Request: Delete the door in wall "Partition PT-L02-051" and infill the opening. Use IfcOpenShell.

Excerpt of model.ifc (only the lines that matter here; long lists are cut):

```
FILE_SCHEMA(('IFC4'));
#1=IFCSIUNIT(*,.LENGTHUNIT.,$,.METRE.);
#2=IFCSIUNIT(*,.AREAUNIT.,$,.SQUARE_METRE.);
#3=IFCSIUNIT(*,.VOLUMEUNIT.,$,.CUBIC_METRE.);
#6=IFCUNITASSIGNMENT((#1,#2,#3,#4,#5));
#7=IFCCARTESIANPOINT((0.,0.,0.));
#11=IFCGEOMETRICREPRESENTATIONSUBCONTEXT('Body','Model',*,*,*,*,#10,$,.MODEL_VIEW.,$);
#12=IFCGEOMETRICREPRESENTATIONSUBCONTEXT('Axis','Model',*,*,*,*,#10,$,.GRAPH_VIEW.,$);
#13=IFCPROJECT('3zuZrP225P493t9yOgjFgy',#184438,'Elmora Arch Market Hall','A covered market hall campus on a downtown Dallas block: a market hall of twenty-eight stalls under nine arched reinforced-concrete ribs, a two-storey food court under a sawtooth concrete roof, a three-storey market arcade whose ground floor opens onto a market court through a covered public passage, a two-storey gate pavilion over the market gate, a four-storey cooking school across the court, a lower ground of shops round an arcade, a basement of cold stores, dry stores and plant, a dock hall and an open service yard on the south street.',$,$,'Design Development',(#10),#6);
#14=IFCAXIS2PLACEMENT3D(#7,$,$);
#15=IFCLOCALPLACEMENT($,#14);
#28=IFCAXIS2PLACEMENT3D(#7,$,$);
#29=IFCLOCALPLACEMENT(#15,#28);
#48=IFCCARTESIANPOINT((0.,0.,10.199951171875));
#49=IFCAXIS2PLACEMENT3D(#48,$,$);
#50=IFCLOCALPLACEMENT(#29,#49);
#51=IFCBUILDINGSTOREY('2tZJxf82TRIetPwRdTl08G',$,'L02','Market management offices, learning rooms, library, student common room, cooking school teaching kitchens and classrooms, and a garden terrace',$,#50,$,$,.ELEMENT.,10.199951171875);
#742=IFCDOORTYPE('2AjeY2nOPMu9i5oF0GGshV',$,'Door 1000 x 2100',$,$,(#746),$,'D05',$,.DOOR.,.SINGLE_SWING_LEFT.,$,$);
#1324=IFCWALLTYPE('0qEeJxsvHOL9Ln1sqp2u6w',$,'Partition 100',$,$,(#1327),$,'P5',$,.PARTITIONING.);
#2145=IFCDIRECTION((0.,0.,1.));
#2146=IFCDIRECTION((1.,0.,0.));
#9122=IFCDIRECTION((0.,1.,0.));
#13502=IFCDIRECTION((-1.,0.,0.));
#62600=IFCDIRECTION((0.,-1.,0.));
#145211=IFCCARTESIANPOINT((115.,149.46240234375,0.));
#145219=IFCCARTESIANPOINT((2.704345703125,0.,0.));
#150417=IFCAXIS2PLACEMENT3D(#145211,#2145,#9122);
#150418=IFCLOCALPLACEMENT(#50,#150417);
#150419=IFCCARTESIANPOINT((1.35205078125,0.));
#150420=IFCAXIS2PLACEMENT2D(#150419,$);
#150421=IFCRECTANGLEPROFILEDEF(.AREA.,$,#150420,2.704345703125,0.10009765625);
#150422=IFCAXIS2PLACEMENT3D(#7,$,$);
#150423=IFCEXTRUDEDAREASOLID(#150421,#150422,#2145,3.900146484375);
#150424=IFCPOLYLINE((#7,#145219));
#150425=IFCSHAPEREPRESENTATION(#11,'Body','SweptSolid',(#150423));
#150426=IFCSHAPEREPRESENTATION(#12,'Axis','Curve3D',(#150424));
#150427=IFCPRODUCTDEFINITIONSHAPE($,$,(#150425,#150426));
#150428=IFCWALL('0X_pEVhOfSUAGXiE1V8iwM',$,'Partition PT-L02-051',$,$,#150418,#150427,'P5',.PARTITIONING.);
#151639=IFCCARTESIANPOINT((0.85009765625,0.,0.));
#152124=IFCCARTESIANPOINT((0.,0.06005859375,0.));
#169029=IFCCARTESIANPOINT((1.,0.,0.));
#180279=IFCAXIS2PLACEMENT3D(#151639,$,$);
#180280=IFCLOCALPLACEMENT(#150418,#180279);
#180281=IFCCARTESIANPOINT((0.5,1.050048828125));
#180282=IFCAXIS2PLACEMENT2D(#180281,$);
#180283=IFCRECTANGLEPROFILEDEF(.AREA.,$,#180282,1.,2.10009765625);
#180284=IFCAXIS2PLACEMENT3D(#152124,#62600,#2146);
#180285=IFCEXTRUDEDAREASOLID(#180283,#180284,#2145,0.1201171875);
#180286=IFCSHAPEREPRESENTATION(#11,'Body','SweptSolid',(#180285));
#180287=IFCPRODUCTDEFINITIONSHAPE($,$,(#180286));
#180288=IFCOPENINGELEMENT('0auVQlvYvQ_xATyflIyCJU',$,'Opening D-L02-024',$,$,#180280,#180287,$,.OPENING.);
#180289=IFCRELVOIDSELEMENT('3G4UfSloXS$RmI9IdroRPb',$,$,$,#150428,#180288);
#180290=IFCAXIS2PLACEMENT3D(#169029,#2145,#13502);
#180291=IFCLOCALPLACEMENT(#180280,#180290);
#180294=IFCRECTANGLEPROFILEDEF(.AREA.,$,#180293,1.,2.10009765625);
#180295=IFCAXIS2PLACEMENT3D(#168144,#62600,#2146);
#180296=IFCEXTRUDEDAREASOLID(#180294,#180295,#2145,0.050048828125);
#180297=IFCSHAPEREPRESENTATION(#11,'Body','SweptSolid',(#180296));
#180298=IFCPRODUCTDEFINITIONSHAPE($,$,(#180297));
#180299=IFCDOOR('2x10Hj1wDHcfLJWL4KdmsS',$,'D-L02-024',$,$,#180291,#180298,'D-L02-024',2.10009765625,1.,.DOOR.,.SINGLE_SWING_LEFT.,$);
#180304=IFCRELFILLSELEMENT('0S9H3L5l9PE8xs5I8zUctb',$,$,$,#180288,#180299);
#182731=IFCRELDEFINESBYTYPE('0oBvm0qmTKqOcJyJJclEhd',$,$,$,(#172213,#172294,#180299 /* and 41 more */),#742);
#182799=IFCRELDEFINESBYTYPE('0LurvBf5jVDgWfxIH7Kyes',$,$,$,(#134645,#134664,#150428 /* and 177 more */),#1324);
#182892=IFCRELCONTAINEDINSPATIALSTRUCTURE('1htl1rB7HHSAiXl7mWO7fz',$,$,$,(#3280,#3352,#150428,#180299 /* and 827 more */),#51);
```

```python
import ifcopenshell
import ifcopenshell.api.feature
import ifcopenshell.api.root
import ifcopenshell.geom
import ifcopenshell.util.shape

model = ifcopenshell.open("model.ifc")
settings = ifcopenshell.geom.settings()


def volume(element):
    """Net volume in cubic metres, openings subtracted."""
    shape = ifcopenshell.geom.create_shape(settings, element)
    return ifcopenshell.util.shape.get_volume(shape.geometry)


door = model.by_id(180299)
opening = door.FillsVoids[0].RelatingOpeningElement
wall = opening.VoidsElements[0].RelatingBuildingElement
before = volume(wall)

ifcopenshell.api.root.remove_product(model, product=door)
ifcopenshell.api.feature.remove_feature(model, feature=opening)

after = volume(wall)

print(f"wall volume {before:.3f} -> {after:.3f} m3")

model.write("model_rev.ifc")
```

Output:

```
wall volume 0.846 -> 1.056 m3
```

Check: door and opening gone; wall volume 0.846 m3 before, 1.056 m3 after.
